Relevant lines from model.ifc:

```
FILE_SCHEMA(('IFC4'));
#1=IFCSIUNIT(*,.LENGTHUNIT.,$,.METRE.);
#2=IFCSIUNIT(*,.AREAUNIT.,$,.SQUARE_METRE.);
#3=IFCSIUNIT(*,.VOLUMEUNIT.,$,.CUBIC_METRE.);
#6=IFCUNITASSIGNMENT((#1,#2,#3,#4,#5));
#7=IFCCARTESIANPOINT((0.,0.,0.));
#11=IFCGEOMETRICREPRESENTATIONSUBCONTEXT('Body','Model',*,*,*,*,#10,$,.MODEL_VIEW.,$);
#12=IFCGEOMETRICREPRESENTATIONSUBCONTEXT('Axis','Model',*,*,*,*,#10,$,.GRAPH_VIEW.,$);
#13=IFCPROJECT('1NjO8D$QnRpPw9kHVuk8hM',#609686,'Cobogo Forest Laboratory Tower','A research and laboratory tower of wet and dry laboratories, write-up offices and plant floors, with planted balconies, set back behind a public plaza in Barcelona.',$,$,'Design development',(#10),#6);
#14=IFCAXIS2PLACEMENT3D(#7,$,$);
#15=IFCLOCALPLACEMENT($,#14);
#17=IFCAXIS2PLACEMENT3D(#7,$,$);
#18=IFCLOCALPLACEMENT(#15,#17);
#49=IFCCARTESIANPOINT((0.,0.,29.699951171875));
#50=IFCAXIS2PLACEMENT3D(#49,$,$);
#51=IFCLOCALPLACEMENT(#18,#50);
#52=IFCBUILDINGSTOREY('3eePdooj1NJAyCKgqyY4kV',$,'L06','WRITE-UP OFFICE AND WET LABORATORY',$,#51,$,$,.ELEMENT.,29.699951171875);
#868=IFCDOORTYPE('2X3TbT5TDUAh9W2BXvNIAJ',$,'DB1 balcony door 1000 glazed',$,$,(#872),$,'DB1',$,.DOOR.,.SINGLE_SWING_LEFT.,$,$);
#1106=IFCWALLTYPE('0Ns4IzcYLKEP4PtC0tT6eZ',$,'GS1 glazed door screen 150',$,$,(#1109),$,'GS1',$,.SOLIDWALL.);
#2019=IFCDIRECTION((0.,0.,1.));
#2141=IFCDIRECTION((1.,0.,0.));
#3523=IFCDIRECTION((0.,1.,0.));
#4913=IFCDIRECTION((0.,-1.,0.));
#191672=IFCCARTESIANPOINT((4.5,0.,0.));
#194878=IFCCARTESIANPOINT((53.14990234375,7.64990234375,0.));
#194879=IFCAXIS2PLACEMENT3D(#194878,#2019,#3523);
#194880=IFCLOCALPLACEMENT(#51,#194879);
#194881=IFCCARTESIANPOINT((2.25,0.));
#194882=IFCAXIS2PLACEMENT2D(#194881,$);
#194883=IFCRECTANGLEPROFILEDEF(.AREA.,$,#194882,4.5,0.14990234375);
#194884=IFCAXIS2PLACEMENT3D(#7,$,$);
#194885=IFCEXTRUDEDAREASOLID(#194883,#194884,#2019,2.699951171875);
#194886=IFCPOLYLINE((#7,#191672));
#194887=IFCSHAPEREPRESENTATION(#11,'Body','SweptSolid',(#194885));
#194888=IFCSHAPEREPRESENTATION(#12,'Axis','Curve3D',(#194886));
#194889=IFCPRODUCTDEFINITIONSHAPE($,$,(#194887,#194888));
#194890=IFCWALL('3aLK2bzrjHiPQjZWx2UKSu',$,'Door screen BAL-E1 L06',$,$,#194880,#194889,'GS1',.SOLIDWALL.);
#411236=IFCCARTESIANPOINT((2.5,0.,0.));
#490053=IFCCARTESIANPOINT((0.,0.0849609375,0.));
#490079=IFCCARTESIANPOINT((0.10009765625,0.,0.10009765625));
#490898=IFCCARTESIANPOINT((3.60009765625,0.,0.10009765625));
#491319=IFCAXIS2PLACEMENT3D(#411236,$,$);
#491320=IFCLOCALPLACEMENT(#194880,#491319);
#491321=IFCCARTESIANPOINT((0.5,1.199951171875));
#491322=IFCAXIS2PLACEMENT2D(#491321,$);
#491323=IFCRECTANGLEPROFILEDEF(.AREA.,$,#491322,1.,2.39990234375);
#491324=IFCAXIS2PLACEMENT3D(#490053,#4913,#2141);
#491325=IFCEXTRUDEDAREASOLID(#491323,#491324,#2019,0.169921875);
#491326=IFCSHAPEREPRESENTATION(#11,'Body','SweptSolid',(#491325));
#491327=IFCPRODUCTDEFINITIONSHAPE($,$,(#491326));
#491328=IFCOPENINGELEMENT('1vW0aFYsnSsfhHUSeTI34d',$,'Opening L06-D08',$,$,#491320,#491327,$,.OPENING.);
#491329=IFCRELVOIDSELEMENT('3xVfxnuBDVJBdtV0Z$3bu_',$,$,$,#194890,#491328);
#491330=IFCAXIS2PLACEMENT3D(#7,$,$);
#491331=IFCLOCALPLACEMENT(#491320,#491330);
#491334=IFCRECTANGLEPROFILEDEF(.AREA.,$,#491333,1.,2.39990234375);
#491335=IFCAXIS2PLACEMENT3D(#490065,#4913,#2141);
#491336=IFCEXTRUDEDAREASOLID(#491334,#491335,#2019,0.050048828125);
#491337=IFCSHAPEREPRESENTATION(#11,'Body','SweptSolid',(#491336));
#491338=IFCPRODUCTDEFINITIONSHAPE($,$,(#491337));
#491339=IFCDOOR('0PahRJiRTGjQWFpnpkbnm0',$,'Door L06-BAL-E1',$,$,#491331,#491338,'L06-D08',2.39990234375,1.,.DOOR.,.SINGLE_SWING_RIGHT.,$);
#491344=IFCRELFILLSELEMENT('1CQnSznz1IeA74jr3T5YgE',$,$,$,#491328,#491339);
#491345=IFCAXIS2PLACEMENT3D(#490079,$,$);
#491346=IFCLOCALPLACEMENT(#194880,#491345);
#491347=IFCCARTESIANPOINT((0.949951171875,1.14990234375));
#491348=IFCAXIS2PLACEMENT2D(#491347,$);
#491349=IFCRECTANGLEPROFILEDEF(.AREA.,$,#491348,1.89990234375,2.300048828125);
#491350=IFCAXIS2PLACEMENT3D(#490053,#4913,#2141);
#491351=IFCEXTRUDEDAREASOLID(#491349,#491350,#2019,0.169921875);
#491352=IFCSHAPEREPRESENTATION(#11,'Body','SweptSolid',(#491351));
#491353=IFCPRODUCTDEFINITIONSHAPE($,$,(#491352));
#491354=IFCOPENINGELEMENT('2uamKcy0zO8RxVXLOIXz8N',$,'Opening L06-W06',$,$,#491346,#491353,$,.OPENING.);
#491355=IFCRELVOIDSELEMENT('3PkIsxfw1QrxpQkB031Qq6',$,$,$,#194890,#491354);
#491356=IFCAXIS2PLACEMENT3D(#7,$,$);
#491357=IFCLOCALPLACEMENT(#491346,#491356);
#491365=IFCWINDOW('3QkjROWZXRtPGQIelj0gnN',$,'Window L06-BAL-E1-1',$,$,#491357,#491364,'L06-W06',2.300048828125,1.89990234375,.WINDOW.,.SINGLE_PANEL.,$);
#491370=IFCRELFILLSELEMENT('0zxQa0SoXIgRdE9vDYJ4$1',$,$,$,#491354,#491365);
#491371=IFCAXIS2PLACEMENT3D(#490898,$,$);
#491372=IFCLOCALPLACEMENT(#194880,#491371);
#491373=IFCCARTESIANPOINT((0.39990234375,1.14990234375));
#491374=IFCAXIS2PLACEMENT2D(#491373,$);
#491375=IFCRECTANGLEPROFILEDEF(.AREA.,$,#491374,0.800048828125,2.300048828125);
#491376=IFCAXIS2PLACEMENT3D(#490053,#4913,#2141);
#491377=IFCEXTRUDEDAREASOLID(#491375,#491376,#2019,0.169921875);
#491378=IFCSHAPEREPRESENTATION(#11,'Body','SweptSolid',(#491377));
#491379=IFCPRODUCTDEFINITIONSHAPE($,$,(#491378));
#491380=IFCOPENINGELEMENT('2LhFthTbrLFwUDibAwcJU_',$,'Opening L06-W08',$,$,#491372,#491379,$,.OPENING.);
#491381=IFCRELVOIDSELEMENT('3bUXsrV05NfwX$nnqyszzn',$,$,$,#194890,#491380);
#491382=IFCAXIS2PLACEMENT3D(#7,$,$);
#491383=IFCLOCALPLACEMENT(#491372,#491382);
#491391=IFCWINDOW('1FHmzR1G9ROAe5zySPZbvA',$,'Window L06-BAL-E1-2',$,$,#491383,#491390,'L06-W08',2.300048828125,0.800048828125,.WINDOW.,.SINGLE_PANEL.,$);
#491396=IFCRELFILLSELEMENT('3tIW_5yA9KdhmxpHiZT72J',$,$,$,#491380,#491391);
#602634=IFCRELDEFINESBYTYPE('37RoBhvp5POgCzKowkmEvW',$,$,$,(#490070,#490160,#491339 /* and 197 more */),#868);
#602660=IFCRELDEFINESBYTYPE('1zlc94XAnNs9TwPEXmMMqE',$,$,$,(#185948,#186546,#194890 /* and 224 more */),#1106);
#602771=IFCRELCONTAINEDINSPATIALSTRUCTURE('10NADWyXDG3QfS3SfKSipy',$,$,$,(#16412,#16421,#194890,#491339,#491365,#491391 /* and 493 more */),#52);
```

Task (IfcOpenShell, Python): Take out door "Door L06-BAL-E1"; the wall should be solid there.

```python
import ifcopenshell
import ifcopenshell.api.feature
import ifcopenshell.api.root
import ifcopenshell.geom
import ifcopenshell.util.shape

model = ifcopenshell.open("model.ifc")
settings = ifcopenshell.geom.settings()


def volume(element):
    """Net volume in cubic metres, openings subtracted."""
    shape = ifcopenshell.geom.create_shape(settings, element)
    return ifcopenshell.util.shape.get_volume(shape.geometry)


door = model.by_guid("0PahRJiRTGjQWFpnpkbnm0")
opening = door.FillsVoids[0].RelatingOpeningElement
wall = opening.VoidsElements[0].RelatingBuildingElement
before = volume(wall)

ifcopenshell.api.root.remove_product(model, product=door)
ifcopenshell.api.feature.remove_feature(model, feature=opening)

after = volume(wall)

print(f"wall volume {before:.3f} -> {after:.3f} m3")

model.write("model_v2.ifc")
```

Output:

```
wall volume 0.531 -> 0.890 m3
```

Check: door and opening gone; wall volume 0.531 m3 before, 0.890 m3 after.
